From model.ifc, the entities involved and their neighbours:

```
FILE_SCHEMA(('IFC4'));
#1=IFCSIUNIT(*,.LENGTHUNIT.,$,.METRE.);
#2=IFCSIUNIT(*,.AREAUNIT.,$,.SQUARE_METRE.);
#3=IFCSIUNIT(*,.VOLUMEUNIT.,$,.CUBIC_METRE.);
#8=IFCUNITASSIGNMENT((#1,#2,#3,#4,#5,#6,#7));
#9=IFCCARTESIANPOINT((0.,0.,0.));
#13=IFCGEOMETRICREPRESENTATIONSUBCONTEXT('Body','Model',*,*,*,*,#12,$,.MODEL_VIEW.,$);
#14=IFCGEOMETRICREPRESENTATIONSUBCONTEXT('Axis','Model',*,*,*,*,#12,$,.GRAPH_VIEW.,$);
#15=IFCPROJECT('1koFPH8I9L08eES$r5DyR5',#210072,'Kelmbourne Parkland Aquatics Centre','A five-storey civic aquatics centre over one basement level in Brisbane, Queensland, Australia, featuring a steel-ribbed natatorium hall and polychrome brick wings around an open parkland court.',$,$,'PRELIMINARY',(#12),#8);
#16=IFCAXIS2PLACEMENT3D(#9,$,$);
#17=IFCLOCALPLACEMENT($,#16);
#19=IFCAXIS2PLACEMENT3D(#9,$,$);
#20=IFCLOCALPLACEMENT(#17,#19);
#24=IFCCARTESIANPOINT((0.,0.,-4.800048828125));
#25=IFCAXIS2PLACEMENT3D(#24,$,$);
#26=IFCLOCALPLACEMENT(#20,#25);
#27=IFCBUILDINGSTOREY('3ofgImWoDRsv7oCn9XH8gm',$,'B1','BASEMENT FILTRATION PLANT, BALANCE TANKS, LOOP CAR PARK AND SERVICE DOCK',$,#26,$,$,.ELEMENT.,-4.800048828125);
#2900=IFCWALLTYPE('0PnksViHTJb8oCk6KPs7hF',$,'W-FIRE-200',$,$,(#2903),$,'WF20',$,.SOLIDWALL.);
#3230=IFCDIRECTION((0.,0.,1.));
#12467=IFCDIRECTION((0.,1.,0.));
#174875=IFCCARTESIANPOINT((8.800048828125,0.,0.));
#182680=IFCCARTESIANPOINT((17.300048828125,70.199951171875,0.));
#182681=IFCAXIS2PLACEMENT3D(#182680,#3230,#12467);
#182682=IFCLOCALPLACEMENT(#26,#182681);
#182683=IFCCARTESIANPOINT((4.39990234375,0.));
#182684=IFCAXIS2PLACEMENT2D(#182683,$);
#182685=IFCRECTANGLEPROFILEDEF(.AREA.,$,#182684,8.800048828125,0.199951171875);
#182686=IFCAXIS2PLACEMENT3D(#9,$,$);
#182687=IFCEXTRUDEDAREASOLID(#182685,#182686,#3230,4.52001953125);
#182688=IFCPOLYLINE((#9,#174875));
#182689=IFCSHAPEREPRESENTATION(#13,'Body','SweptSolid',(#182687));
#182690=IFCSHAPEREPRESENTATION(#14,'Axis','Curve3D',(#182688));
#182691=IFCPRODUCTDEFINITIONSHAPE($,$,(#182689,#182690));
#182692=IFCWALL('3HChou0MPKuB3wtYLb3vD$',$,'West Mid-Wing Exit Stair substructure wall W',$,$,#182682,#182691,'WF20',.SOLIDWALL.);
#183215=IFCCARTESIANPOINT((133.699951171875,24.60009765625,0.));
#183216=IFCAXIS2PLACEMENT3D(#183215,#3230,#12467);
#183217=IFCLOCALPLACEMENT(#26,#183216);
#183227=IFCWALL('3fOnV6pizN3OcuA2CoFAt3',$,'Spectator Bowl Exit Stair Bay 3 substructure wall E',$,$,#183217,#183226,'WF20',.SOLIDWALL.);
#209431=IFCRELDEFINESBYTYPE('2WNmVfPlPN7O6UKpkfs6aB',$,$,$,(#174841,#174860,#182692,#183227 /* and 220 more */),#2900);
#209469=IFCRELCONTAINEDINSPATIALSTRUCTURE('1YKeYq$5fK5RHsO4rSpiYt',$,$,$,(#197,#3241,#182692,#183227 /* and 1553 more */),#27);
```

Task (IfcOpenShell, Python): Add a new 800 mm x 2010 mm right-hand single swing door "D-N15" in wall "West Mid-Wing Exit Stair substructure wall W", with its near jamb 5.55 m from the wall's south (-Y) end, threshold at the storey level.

```python
import numpy as np
import ifcopenshell
import ifcopenshell.api.feature
import ifcopenshell.api.geometry
import ifcopenshell.api.root
import ifcopenshell.api.spatial
import ifcopenshell.geom
import ifcopenshell.util.element
import ifcopenshell.util.placement
import ifcopenshell.util.representation
import ifcopenshell.util.shape
import ifcopenshell.util.unit

model = ifcopenshell.open("model.ifc")
unit_scale = ifcopenshell.util.unit.calculate_unit_scale(model)
settings = ifcopenshell.geom.settings()


def volume(element):
    """Net volume in cubic metres, openings subtracted."""
    shape = ifcopenshell.geom.create_shape(settings, element)
    return ifcopenshell.util.shape.get_volume(shape.geometry)


wall = model.by_guid("3HChou0MPKuB3wtYLb3vD$")
storey = ifcopenshell.util.element.get_container(wall, ifc_class="IfcBuildingStorey")
context = ifcopenshell.util.representation.get_context(model, "Model", "Body", "MODEL_VIEW")
before = volume(wall)

width, height, from_end, sill = 0.8, 2.01, 5.55, 0.0  # metres

# The wall runs along its own X axis, and the end named is its -X end.
wall_shape = ifcopenshell.geom.create_shape(settings, wall)
x, y, z = ifcopenshell.util.shape.get_vertices(wall_shape.geometry).T
start = x.min() + from_end
face, thickness = float(y.min()), float(y.max() - y.min())
wall_matrix = ifcopenshell.util.placement.get_local_placement(wall.ObjectPlacement)
level = ifcopenshell.util.placement.get_local_placement(storey.ObjectPlacement)[2, 3]


def in_wall(x, y):
    """Placement at x, y metres in the wall's axes, at sill height."""
    matrix = wall_matrix.copy()
    matrix[:, 3] = wall_matrix @ np.array([x / unit_scale, y / unit_scale, 0.0, 1.0])
    matrix[2, 3] = level + sill / unit_scale
    return matrix


# Opening: a box that overshoots both wall faces by 50 mm.
opening = ifcopenshell.api.root.create_entity(model, ifc_class="IfcOpeningElement", predefined_type="OPENING")
box = ifcopenshell.api.geometry.add_wall_representation(
    model, context=context, length=width, height=height, thickness=thickness + 0.1
)
ifcopenshell.api.geometry.assign_representation(model, product=opening, representation=box)
ifcopenshell.api.geometry.edit_object_placement(model, product=opening, matrix=in_wall(start, face - 0.05), is_si=False)
ifcopenshell.api.feature.add_feature(model, feature=opening, element=wall)

door = ifcopenshell.api.root.create_entity(model, ifc_class="IfcDoor", name="D-N15", predefined_type="DOOR")
door.OverallWidth, door.OverallHeight = width / unit_scale, height / unit_scale
door.OperationType = "SINGLE_SWING_RIGHT"
body = ifcopenshell.api.geometry.add_door_representation(
    model,
    context=context,
    overall_width=door.OverallWidth,
    overall_height=door.OverallHeight,
    operation_type="SINGLE_SWING_RIGHT",
    lining_properties={"LiningDepth": thickness / unit_scale, "ThresholdDepth": thickness / unit_scale},
)
ifcopenshell.api.geometry.assign_representation(model, product=door, representation=body)
ifcopenshell.api.spatial.assign_container(model, products=[door], relating_structure=storey)
ifcopenshell.api.feature.add_filling(model, opening=opening, element=door)

# The lining spans the wall, so the door starts at the wall face.
ifcopenshell.api.geometry.edit_object_placement(model, product=door, matrix=in_wall(start, face), is_si=False)

after = volume(wall)

print(f"wall volume {before:.3f} -> {after:.3f} m3")

model.write("model-out.ifc")
```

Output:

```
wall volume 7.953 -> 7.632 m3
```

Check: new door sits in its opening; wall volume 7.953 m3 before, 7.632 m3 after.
